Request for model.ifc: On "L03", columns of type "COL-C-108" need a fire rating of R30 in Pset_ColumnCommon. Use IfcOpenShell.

First a look at what the model holds.

```python
import ifcopenshell
import ifcopenshell.util.element

model = ifcopenshell.open("model.ifc")
print(model.schema)
storey = next(s for s in model.by_type("IfcBuildingStorey") if s.Name == "L03")
columns = [e for e in ifcopenshell.util.element.get_decomposition(storey) if e.is_a("IfcColumn")]
seen = {}
for e in columns:
    element_type = ifcopenshell.util.element.get_type(e)
    key = (element_type.Name if element_type != e and element_type else None, ifcopenshell.util.element.get_pset(e, "Pset_ColumnCommon", "FireRating"))
    seen[key] = seen.get(key, 0) + 1
for (name, value), count in sorted(seen.items(), key=str):
    print(count, "x", name, "|", value)
```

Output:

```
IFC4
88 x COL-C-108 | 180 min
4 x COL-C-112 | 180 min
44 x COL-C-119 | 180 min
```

```python
import ifcopenshell
import ifcopenshell.api.pset
import ifcopenshell.util.element

model = ifcopenshell.open("model.ifc")

storey = next(s for s in model.by_type("IfcBuildingStorey") if s.Name == "L03")
columns = [e for e in ifcopenshell.util.element.get_decomposition(storey) if e.is_a("IfcColumn")]

count = 0
for e in columns:
    element_type = ifcopenshell.util.element.get_type(e)
    if element_type in (None, e) or element_type.Name != "COL-C-108":
        continue
    # add_pset returns the element's existing set when there is one.
    pset = ifcopenshell.api.pset.add_pset(model, product=e, name="Pset_ColumnCommon")
    ifcopenshell.api.pset.edit_pset(model, pset=pset, properties={"FireRating": "R30"})
    count += 1

print(count, "columns updated")

model.write("model_updated.ifc")
```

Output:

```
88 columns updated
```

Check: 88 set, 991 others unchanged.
